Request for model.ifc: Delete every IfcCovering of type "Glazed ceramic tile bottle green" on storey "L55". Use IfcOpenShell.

First a look at what the model holds.

```python
import ifcopenshell
import ifcopenshell.util.element

model = ifcopenshell.open("model.ifc")
print(model.schema)
storey = next(s for s in model.by_type("IfcBuildingStorey") if s.Name == "L55")
coverings = [e for e in ifcopenshell.util.element.get_decomposition(storey) if e.is_a("IfcCovering")]
seen = {}
for e in coverings:
    element_type = ifcopenshell.util.element.get_type(e)
    name = element_type.Name if element_type not in (None, e) else None
    seen[name] = seen.get(name, 0) + 1
for name, count in sorted(seen.items(), key=str):
    print(count, "x", name)
```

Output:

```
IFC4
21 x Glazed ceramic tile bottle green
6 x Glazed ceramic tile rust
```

```python
import ifcopenshell
import ifcopenshell.api.root
import ifcopenshell.util.element

model = ifcopenshell.open("model.ifc")

storey = next(s for s in model.by_type("IfcBuildingStorey") if s.Name == "L55")
coverings = [e for e in ifcopenshell.util.element.get_decomposition(storey) if e.is_a("IfcCovering")]
targets = [e for e in coverings if (t := ifcopenshell.util.element.get_type(e)) not in (None, e) and t.Name == "Glazed ceramic tile bottle green"]

for e in targets:
    ifcopenshell.api.root.remove_product(model, product=e)
print(len(targets), "removed")

model.write("model_v2.ifc")
```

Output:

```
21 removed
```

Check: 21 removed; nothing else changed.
